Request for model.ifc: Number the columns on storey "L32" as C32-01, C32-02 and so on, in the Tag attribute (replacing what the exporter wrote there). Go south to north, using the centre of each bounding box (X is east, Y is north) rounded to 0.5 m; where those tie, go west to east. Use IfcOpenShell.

First a look at what the model holds.

```python
import ifcopenshell
import ifcopenshell.util.element
import ifcopenshell.util.placement

model = ifcopenshell.open("model.ifc")
print(model.schema)
storey = next(s for s in model.by_type("IfcBuildingStorey") if s.Name == "L32")
columns = [e for e in ifcopenshell.util.element.get_decomposition(storey) if e.is_a("IfcColumn")]
for e in sorted(columns, key=lambda e: e.id()):
    origin = ifcopenshell.util.placement.get_local_placement(e.ObjectPlacement)[:3, 3]
    print(e.id(), e.Tag, e.Name, origin.round(2) + 0.0, sep=" | ")
```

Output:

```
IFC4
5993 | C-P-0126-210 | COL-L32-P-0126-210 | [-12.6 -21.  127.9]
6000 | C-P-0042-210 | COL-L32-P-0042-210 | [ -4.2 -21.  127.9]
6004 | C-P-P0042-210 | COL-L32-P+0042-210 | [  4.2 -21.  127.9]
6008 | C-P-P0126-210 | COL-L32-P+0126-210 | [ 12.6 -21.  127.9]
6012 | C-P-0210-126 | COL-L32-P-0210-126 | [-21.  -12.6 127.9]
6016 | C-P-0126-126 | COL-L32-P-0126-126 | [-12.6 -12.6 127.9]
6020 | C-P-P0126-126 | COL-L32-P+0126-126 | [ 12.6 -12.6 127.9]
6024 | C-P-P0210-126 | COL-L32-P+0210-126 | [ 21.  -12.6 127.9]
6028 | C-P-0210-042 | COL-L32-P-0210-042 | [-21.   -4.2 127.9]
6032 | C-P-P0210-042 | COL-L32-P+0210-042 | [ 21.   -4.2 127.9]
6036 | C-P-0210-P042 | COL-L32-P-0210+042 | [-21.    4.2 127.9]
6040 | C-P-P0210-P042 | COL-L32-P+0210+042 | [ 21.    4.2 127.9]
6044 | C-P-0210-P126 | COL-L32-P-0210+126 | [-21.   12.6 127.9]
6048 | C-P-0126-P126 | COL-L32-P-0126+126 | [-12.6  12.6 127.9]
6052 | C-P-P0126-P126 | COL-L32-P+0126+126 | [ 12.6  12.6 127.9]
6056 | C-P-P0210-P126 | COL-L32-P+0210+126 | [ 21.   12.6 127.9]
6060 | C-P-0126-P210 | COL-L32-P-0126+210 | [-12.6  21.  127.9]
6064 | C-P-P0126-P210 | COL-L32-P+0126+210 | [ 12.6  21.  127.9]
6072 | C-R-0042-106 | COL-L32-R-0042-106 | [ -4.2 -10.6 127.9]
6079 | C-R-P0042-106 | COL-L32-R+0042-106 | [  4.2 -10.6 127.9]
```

```python
import ifcopenshell
import ifcopenshell.geom
import ifcopenshell.util.element
import ifcopenshell.util.shape

model = ifcopenshell.open("model.ifc")
settings = ifcopenshell.geom.settings()
settings.set("use-world-coords", True)


def centre(element):
    shape = ifcopenshell.geom.create_shape(settings, element)
    return ifcopenshell.util.shape.get_bbox_centroid(shape.geometry)


storey = next(s for s in model.by_type("IfcBuildingStorey") if s.Name == "L32")
columns = [e for e in ifcopenshell.util.element.get_decomposition(storey) if e.is_a("IfcColumn")]

# Insertion points can sit at a corner or the storey origin, so sort by the geometry (in metres).
centres = {e: centre(e) for e in columns}
columns.sort(key=lambda e: (round(centres[e][1] / 0.5), centres[e][0]))

for i, e in enumerate(columns, start=1):
    number = f"C32-{i:02d}"
    e.Tag = number
    print(e.id(), number)

model.write("model_rev.ifc")
```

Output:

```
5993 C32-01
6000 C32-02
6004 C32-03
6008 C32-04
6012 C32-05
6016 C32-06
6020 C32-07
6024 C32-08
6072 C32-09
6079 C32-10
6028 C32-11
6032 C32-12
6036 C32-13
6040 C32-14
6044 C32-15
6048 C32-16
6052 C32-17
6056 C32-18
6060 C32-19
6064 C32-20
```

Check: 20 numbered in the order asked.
